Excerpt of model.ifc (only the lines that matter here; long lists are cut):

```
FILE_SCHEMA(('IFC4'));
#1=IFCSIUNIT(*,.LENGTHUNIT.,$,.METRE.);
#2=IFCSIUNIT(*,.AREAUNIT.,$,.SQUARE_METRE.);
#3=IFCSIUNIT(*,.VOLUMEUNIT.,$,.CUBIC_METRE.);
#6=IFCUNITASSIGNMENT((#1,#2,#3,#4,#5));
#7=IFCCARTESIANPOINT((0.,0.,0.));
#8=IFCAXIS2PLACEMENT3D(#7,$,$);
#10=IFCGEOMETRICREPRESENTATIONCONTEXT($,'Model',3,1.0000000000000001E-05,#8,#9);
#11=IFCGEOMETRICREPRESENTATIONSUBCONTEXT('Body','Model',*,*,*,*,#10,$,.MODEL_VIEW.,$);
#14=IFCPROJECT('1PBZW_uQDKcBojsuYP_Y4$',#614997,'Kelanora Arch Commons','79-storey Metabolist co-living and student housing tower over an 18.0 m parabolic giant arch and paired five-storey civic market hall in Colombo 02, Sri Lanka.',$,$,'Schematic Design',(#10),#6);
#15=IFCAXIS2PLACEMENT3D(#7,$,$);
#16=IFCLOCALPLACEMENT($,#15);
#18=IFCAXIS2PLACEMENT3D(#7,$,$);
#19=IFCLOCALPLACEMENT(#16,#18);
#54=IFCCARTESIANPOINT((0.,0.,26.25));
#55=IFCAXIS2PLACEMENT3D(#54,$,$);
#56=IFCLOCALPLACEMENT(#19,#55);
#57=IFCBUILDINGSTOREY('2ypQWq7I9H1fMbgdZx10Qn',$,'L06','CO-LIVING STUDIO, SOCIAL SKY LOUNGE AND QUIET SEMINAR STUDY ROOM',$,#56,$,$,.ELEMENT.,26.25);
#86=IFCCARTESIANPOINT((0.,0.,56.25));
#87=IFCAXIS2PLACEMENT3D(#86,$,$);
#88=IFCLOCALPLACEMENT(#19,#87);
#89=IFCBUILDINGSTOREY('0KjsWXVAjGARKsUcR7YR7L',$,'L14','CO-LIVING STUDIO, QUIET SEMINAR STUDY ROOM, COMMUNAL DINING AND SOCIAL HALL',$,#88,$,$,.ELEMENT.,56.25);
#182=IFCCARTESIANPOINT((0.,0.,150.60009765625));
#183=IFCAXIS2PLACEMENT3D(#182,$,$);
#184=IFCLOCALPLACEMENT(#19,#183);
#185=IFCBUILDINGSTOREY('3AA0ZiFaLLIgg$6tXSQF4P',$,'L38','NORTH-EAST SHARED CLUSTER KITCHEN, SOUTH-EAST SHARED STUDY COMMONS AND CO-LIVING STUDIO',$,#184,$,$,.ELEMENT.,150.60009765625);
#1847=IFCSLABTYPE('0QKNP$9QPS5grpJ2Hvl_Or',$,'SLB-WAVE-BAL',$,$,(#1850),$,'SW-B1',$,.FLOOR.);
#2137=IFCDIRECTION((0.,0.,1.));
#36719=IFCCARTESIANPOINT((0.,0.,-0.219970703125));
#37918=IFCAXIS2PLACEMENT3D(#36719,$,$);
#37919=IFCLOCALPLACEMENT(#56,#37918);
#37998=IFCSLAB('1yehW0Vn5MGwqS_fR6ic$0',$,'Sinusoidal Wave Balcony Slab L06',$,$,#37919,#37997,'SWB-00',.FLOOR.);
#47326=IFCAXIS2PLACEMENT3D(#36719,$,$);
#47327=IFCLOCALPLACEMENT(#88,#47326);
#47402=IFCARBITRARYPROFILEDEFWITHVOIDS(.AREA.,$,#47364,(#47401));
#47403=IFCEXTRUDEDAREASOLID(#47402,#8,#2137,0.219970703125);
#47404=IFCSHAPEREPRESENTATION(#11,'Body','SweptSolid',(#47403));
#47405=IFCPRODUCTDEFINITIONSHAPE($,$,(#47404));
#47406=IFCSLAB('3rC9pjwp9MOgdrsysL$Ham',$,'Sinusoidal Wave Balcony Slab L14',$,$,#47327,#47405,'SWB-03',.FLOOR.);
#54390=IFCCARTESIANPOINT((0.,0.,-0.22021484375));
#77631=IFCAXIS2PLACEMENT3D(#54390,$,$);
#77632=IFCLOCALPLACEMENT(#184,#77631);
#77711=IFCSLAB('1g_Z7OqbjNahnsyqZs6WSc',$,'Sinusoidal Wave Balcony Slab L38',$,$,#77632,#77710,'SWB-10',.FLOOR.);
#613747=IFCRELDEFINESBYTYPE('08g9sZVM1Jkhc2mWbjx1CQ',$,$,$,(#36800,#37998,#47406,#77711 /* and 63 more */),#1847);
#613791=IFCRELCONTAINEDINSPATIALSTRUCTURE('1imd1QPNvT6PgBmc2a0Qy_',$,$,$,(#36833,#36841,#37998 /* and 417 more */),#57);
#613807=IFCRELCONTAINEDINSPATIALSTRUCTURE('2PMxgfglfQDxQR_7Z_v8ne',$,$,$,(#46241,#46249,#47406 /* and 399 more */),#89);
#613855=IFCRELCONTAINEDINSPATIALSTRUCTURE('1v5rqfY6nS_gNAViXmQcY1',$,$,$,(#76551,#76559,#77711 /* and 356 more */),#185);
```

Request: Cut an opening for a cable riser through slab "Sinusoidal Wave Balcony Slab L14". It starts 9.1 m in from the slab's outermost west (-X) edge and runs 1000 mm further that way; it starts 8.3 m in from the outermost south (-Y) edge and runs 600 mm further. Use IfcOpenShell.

```python
import numpy as np
import ifcopenshell
import ifcopenshell.api.feature
import ifcopenshell.api.geometry
import ifcopenshell.api.root
import ifcopenshell.geom
import ifcopenshell.util.placement
import ifcopenshell.util.representation
import ifcopenshell.util.shape
import ifcopenshell.util.unit

model = ifcopenshell.open("model.ifc")
unit_scale = ifcopenshell.util.unit.calculate_unit_scale(model)
settings = ifcopenshell.geom.settings()


def volume(element):
    """Net volume in cubic metres, openings subtracted."""
    shape = ifcopenshell.geom.create_shape(settings, element)
    return ifcopenshell.util.shape.get_volume(shape.geometry)


slab = model.by_guid("3rC9pjwp9MOgdrsysL$Ham")
before = volume(slab)

# Extent in the slab's own axes, in metres. The edges named are its -X and -Y sides.
slab_shape = ifcopenshell.geom.create_shape(settings, slab)
vertices = ifcopenshell.util.shape.get_vertices(slab_shape.geometry)
x_min, y_min, bottom = vertices.min(axis=0)
top = vertices[:, 2].max()

opening = ifcopenshell.api.root.create_entity(model, ifc_class="IfcOpeningElement", name="Cable riser opening", predefined_type="OPENING")
context = ifcopenshell.util.representation.get_context(model, "Model", "Body", "MODEL_VIEW")
width, depth = 1, 0.6
outline = [(0.0, 0.0), (width, 0.0), (width, depth), (0.0, depth), (0.0, 0.0)]
# Overshoot both faces by 50 mm so the cut is clean.
shape = ifcopenshell.api.geometry.add_slab_representation(
    model, context=context, depth=top - bottom + 0.1, polyline=outline
)
ifcopenshell.api.geometry.assign_representation(model, product=opening, representation=shape)

matrix = ifcopenshell.util.placement.get_local_placement(slab.ObjectPlacement)
matrix[:, 3] = matrix @ np.append(np.array([x_min + 9.1, y_min + 8.3, bottom - 0.05]) / unit_scale, 1.0)
ifcopenshell.api.geometry.edit_object_placement(model, product=opening, matrix=matrix, is_si=False)
ifcopenshell.api.feature.add_feature(model, feature=opening, element=slab)

after = volume(slab)

print(f"slab volume {before:.3f} -> {after:.3f} m3")

model.write("model_edited.ifc")
```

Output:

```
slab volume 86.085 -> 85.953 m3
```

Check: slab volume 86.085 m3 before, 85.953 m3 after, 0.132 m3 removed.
